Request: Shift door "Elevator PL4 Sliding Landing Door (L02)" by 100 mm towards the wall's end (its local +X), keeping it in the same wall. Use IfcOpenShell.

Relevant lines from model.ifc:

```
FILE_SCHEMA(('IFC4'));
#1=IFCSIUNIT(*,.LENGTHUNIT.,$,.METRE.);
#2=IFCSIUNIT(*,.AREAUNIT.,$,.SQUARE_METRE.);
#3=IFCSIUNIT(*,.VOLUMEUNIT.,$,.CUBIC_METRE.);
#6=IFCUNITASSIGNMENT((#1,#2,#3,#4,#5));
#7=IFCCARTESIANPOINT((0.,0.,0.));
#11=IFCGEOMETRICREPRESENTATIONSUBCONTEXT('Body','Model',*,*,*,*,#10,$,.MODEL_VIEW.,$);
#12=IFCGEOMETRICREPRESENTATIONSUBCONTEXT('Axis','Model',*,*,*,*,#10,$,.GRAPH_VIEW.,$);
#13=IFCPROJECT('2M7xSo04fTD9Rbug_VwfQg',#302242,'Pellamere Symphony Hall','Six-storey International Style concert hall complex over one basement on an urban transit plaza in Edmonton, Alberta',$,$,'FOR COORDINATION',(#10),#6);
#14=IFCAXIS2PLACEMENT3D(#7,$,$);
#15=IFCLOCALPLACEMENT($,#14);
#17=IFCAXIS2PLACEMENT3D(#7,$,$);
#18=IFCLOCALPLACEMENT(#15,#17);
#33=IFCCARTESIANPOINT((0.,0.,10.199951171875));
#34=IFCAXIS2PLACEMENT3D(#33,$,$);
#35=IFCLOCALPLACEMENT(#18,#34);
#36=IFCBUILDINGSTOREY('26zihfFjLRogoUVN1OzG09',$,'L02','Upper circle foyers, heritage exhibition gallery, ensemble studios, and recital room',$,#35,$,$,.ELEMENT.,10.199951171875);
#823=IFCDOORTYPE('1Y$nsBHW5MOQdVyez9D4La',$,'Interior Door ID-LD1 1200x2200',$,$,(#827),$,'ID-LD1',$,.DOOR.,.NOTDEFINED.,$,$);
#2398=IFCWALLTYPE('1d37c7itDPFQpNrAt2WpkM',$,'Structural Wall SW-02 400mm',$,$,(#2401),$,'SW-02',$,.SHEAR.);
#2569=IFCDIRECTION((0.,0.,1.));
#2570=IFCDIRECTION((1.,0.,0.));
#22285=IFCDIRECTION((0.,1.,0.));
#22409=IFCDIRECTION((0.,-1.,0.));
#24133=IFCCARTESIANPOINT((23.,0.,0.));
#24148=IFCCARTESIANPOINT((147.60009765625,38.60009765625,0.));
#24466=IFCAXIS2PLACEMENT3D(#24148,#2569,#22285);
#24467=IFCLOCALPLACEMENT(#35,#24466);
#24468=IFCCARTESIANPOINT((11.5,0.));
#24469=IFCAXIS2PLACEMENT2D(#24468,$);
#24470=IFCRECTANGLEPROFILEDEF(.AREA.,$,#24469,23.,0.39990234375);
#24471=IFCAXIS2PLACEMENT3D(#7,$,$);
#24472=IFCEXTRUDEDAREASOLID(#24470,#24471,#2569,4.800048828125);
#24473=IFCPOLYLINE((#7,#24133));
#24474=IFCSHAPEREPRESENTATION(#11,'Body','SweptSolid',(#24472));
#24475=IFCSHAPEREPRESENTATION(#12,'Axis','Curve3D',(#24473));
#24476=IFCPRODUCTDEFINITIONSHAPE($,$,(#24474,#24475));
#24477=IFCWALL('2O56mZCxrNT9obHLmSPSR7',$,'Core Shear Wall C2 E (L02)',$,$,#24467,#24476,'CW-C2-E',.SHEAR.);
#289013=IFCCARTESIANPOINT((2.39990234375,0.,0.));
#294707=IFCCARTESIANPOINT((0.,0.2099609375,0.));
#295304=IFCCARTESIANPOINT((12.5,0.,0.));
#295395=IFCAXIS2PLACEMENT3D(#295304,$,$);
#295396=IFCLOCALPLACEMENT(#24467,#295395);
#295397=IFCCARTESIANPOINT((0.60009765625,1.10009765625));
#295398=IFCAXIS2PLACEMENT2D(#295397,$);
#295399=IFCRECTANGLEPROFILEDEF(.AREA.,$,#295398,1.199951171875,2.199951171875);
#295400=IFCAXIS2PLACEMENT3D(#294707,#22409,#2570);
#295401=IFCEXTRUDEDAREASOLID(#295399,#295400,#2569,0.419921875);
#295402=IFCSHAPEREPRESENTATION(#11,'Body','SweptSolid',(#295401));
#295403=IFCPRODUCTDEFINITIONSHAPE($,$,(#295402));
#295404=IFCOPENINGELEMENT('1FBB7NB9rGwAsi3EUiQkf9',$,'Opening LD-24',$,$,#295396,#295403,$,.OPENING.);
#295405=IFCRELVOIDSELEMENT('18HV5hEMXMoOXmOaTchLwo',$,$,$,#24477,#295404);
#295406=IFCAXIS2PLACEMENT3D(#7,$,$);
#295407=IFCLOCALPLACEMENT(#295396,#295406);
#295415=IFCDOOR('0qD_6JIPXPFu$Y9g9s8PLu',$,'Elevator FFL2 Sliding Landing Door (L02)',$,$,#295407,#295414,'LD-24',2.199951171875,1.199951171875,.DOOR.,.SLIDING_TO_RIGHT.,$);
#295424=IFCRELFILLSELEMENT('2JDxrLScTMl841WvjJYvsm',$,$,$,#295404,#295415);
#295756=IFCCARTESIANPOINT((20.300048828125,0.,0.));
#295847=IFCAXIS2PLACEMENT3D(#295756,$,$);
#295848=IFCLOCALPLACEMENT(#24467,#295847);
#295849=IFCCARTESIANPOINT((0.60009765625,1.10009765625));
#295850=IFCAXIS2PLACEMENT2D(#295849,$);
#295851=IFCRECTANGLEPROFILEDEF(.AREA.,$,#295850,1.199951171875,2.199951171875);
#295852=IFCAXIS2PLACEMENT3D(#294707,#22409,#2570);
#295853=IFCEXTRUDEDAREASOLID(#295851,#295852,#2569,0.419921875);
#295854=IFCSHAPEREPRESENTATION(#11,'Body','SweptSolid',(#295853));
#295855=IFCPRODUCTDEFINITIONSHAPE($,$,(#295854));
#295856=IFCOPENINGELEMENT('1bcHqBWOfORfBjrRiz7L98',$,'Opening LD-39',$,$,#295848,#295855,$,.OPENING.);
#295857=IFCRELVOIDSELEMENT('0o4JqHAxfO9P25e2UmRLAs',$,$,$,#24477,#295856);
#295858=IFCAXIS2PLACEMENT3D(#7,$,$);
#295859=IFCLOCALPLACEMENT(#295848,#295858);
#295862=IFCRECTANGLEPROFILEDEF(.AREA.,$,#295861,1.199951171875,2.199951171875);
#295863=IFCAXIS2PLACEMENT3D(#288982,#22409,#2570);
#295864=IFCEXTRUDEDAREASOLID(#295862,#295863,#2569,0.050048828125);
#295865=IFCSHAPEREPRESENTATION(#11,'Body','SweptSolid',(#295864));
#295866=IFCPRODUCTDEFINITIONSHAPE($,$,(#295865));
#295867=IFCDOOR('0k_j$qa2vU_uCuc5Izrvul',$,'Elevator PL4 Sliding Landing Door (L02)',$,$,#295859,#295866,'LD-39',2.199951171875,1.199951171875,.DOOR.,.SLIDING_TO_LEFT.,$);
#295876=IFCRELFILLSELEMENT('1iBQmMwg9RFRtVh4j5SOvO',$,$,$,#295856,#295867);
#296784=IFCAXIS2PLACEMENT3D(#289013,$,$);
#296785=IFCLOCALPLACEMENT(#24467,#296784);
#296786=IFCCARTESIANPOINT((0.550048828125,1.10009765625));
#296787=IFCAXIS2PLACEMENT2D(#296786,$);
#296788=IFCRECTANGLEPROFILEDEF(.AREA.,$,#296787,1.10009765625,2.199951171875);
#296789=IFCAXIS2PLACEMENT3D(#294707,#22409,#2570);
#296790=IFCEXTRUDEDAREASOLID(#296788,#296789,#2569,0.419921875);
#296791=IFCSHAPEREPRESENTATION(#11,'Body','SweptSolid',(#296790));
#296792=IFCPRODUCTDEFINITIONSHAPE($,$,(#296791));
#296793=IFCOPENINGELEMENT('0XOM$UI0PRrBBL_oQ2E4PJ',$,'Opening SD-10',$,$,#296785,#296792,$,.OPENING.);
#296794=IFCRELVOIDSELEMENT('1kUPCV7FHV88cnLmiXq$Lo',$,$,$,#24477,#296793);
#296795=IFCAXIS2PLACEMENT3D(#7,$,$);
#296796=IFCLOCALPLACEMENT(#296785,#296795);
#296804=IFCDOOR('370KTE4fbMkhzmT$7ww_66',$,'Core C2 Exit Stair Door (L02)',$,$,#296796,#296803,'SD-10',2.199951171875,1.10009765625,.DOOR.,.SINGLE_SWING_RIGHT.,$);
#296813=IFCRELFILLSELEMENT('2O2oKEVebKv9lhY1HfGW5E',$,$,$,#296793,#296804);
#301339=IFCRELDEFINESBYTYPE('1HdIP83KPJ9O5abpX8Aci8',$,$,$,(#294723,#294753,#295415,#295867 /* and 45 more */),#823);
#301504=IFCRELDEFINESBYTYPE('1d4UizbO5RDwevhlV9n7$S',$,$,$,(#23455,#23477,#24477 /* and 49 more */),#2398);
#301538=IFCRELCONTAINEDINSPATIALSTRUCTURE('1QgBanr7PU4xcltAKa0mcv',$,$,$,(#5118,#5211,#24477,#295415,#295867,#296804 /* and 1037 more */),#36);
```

```python
import ifcopenshell
import ifcopenshell.api.geometry
import ifcopenshell.util.placement

model = ifcopenshell.open("model.ifc")

door = model.by_id(295867)
opening = door.FillsVoids[0].RelatingOpeningElement
wall = opening.VoidsElements[0].RelatingBuildingElement

wall_matrix = ifcopenshell.util.placement.get_local_placement(wall.ObjectPlacement)
shift = wall_matrix[:3, 0] * 0.1
before = ifcopenshell.util.placement.get_local_placement(door.ObjectPlacement)[:3, 3].copy()

# The door is placed relative to its opening, so it follows when the opening moves.
matrix = ifcopenshell.util.placement.get_local_placement(opening.ObjectPlacement)
matrix[:3, 3] += shift
ifcopenshell.api.geometry.edit_object_placement(
    model, product=opening, matrix=matrix, is_si=False, should_transform_children=True
)

after = ifcopenshell.util.placement.get_local_placement(door.ObjectPlacement)[:3, 3]
print("door moved by", (after - before).round(3) + 0.0)

model.write("model_updated.ifc")
```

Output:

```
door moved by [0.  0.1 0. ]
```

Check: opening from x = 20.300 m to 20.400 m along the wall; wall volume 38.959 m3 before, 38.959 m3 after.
